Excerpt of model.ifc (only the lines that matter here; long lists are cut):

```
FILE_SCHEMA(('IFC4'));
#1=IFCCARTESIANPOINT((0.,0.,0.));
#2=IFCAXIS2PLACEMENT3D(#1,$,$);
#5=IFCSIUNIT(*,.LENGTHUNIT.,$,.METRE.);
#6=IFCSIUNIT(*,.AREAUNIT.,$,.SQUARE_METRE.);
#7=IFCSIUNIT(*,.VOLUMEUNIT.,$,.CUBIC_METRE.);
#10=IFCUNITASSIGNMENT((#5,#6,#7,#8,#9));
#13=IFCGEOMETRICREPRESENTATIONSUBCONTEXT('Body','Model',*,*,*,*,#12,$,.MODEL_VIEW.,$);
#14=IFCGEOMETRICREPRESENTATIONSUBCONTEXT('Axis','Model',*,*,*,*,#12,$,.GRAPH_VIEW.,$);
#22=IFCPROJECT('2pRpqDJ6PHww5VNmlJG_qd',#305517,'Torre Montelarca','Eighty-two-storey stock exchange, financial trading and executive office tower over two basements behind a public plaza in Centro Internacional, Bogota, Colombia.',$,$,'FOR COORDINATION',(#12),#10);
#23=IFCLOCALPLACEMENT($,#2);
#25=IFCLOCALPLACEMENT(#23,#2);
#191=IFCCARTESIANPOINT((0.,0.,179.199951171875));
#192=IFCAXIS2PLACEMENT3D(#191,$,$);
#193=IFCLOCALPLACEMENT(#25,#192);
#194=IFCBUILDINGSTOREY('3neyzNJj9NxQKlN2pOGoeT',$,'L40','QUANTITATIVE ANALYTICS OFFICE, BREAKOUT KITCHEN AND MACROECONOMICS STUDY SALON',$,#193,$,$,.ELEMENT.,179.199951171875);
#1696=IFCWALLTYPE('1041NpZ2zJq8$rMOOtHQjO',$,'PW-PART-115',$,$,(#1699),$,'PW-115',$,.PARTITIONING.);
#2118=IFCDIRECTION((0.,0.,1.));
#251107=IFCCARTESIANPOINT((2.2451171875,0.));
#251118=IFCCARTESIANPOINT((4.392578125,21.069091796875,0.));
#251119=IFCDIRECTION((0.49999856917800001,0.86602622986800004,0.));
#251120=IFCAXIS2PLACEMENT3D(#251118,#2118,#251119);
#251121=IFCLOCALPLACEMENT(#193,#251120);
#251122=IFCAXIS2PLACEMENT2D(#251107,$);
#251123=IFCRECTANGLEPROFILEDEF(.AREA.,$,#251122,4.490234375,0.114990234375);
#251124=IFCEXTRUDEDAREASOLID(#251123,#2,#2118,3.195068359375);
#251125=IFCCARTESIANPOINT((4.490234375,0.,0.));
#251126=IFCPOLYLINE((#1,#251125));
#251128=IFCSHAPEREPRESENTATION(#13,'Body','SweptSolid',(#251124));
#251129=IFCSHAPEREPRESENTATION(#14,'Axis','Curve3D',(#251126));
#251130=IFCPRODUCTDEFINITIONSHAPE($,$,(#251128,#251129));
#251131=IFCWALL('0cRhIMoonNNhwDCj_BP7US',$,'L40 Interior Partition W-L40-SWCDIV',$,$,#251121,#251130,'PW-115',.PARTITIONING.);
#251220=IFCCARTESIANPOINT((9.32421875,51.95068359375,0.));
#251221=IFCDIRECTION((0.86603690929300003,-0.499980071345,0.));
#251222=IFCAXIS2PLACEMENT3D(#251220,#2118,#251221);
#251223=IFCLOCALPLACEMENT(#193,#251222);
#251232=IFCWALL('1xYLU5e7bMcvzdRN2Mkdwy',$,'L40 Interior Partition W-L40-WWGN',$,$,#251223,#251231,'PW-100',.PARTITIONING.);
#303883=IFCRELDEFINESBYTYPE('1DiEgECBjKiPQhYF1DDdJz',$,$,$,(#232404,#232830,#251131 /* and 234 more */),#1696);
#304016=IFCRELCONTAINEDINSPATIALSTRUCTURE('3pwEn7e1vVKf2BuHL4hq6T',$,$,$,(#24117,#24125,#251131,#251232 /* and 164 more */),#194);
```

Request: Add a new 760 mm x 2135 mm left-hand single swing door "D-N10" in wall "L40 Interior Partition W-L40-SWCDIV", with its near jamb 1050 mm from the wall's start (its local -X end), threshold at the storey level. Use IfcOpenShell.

```python
import numpy as np
import ifcopenshell
import ifcopenshell.api.feature
import ifcopenshell.api.geometry
import ifcopenshell.api.root
import ifcopenshell.api.spatial
import ifcopenshell.geom
import ifcopenshell.util.element
import ifcopenshell.util.placement
import ifcopenshell.util.representation
import ifcopenshell.util.shape
import ifcopenshell.util.unit

model = ifcopenshell.open("model.ifc")
unit_scale = ifcopenshell.util.unit.calculate_unit_scale(model)
settings = ifcopenshell.geom.settings()


def volume(element):
    """Net volume in cubic metres, openings subtracted."""
    shape = ifcopenshell.geom.create_shape(settings, element)
    return ifcopenshell.util.shape.get_volume(shape.geometry)


wall = model.by_id(251131)
storey = ifcopenshell.util.element.get_container(wall, ifc_class="IfcBuildingStorey")
context = ifcopenshell.util.representation.get_context(model, "Model", "Body", "MODEL_VIEW")
before = volume(wall)

width, height, from_end, sill = 0.76, 2.135, 1.05, 0.0  # metres

# The wall runs along its own X axis, and the end named is its -X end.
wall_shape = ifcopenshell.geom.create_shape(settings, wall)
x, y, z = ifcopenshell.util.shape.get_vertices(wall_shape.geometry).T
start = x.min() + from_end
face, thickness = float(y.min()), float(y.max() - y.min())
wall_matrix = ifcopenshell.util.placement.get_local_placement(wall.ObjectPlacement)
level = ifcopenshell.util.placement.get_local_placement(storey.ObjectPlacement)[2, 3]


def in_wall(x, y):
    """Placement at x, y metres in the wall's axes, at sill height."""
    matrix = wall_matrix.copy()
    matrix[:, 3] = wall_matrix @ np.array([x / unit_scale, y / unit_scale, 0.0, 1.0])
    matrix[2, 3] = level + sill / unit_scale
    return matrix


# Opening: a box that overshoots both wall faces by 50 mm.
opening = ifcopenshell.api.root.create_entity(model, ifc_class="IfcOpeningElement", predefined_type="OPENING")
box = ifcopenshell.api.geometry.add_wall_representation(
    model, context=context, length=width, height=height, thickness=thickness + 0.1
)
ifcopenshell.api.geometry.assign_representation(model, product=opening, representation=box)
ifcopenshell.api.geometry.edit_object_placement(model, product=opening, matrix=in_wall(start, face - 0.05), is_si=False)
ifcopenshell.api.feature.add_feature(model, feature=opening, element=wall)

door = ifcopenshell.api.root.create_entity(model, ifc_class="IfcDoor", name="D-N10", predefined_type="DOOR")
door.OverallWidth, door.OverallHeight = width / unit_scale, height / unit_scale
door.OperationType = "SINGLE_SWING_LEFT"
body = ifcopenshell.api.geometry.add_door_representation(
    model,
    context=context,
    overall_width=door.OverallWidth,
    overall_height=door.OverallHeight,
    operation_type="SINGLE_SWING_LEFT",
    lining_properties={"LiningDepth": thickness / unit_scale, "ThresholdDepth": thickness / unit_scale},
)
ifcopenshell.api.geometry.assign_representation(model, product=door, representation=body)
ifcopenshell.api.spatial.assign_container(model, products=[door], relating_structure=storey)
ifcopenshell.api.feature.add_filling(model, opening=opening, element=door)

# The lining spans the wall, so the door starts at the wall face.
ifcopenshell.api.geometry.edit_object_placement(model, product=door, matrix=in_wall(start, face), is_si=False)

after = volume(wall)

print(f"wall volume {before:.3f} -> {after:.3f} m3")

model.write("model_edited.ifc")
```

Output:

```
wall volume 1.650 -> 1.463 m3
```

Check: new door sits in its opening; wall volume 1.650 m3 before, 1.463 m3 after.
